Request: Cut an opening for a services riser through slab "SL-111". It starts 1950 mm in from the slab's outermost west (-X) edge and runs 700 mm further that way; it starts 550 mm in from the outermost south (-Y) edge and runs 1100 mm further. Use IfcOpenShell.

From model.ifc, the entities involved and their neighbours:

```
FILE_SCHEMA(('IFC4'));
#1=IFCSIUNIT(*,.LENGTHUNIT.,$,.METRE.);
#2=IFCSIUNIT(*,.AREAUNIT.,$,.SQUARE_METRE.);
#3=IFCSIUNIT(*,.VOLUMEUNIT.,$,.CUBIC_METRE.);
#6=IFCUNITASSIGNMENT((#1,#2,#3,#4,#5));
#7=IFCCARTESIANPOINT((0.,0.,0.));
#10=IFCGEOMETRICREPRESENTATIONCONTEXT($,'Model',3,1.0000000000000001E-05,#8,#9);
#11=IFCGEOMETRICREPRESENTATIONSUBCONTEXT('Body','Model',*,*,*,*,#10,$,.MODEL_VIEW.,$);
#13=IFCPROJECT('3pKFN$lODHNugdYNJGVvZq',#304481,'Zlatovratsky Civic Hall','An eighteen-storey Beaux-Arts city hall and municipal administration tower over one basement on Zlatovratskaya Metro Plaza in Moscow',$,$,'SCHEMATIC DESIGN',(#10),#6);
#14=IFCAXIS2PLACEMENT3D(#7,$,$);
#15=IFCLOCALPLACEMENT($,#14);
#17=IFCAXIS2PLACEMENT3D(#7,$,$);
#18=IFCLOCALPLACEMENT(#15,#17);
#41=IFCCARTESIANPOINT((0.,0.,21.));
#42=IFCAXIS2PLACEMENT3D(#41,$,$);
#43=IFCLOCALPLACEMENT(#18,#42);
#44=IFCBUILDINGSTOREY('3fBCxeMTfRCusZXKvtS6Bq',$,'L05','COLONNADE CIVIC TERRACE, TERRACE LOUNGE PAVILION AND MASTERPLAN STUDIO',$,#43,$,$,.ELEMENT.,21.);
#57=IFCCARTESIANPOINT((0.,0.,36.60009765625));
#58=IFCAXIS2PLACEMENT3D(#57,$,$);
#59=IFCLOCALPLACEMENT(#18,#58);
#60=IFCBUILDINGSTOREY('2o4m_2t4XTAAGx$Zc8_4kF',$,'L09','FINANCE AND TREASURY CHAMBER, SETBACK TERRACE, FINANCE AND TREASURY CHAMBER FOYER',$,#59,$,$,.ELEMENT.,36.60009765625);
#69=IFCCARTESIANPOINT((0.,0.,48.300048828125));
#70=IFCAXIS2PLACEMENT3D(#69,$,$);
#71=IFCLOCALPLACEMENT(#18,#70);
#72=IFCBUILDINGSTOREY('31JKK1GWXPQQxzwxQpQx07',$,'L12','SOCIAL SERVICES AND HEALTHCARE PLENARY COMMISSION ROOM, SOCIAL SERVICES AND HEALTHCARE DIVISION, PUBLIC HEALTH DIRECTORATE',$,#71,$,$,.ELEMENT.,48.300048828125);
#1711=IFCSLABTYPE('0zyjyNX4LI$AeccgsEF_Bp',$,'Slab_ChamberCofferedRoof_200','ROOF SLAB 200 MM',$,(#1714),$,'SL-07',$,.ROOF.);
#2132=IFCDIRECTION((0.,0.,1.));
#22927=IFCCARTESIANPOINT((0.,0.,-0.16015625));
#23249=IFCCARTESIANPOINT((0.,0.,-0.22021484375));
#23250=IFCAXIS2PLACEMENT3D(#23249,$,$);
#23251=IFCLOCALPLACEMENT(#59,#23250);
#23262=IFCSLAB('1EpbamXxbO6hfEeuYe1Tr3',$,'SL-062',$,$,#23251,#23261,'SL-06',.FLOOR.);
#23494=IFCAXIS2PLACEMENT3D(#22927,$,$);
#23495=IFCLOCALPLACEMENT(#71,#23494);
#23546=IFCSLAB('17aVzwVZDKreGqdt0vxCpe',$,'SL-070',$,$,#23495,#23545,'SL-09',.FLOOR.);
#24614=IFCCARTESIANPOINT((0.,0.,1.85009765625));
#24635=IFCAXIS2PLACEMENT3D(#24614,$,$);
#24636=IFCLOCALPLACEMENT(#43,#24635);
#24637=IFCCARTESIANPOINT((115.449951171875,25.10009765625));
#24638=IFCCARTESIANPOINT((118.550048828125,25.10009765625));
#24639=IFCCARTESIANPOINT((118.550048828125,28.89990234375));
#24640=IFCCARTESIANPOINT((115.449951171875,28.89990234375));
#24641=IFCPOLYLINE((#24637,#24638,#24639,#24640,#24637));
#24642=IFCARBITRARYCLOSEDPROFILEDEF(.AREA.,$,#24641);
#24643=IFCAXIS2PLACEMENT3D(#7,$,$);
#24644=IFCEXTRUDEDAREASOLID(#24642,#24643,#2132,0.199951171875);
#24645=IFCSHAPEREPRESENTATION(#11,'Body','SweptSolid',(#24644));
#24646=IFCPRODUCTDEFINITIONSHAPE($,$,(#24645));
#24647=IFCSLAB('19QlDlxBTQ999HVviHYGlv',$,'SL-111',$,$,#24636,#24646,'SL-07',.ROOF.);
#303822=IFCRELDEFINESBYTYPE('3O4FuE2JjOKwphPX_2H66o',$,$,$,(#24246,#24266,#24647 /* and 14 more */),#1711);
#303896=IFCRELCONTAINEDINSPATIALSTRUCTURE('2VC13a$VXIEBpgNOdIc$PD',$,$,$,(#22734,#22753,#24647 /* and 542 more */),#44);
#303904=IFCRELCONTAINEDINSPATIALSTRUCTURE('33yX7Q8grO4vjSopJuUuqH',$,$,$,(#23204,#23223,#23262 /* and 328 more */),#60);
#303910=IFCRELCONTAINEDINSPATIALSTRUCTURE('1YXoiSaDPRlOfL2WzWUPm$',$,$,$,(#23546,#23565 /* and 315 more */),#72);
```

```python
import numpy as np
import ifcopenshell
import ifcopenshell.api.feature
import ifcopenshell.api.geometry
import ifcopenshell.api.root
import ifcopenshell.geom
import ifcopenshell.util.placement
import ifcopenshell.util.representation
import ifcopenshell.util.shape
import ifcopenshell.util.unit

model = ifcopenshell.open("model.ifc")
unit_scale = ifcopenshell.util.unit.calculate_unit_scale(model)
settings = ifcopenshell.geom.settings()


def volume(element):
    """Net volume in cubic metres, openings subtracted."""
    shape = ifcopenshell.geom.create_shape(settings, element)
    return ifcopenshell.util.shape.get_volume(shape.geometry)


slab = model.by_guid("19QlDlxBTQ999HVviHYGlv")
before = volume(slab)

# Extent in the slab's own axes, in metres. The edges named are its -X and -Y sides.
slab_shape = ifcopenshell.geom.create_shape(settings, slab)
vertices = ifcopenshell.util.shape.get_vertices(slab_shape.geometry)
x_min, y_min, bottom = vertices.min(axis=0)
top = vertices[:, 2].max()

opening = ifcopenshell.api.root.create_entity(model, ifc_class="IfcOpeningElement", name="Services riser opening", predefined_type="OPENING")
context = ifcopenshell.util.representation.get_context(model, "Model", "Body", "MODEL_VIEW")
width, depth = 0.7, 1.1
outline = [(0.0, 0.0), (width, 0.0), (width, depth), (0.0, depth), (0.0, 0.0)]
# Overshoot both faces by 50 mm so the cut is clean.
shape = ifcopenshell.api.geometry.add_slab_representation(
    model, context=context, depth=top - bottom + 0.1, polyline=outline
)
ifcopenshell.api.geometry.assign_representation(model, product=opening, representation=shape)

matrix = ifcopenshell.util.placement.get_local_placement(slab.ObjectPlacement)
matrix[:, 3] = matrix @ np.append(np.array([x_min + 1.95, y_min + 0.55, bottom - 0.05]) / unit_scale, 1.0)
ifcopenshell.api.geometry.edit_object_placement(model, product=opening, matrix=matrix, is_si=False)
ifcopenshell.api.feature.add_feature(model, feature=opening, element=slab)

after = volume(slab)

print(f"slab volume {before:.3f} -> {after:.3f} m3")

model.write("model_v2.ifc")
```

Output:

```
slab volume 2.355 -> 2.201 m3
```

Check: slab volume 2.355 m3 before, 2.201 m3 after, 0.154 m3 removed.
